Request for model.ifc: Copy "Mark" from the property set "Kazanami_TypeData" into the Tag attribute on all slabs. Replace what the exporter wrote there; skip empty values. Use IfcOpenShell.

First a look at what the model holds.

```python
import ifcopenshell
import ifcopenshell.util.element

model = ifcopenshell.open("model.ifc")
print(model.schema)
slabs = model.by_type("IfcSlab")
print(len(slabs), "slabs")
for e in slabs[:8]:
    source = ifcopenshell.util.element.get_pset(e, "Kazanami_TypeData", "Mark")
    target = e.Tag
    print(e.id(), repr(source), repr(target), sep=" | ")
```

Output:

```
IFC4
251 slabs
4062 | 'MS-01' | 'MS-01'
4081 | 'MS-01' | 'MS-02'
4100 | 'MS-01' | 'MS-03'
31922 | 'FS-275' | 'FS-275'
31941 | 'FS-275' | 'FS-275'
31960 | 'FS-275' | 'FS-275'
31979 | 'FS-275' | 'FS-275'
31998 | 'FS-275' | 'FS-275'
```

```python
import ifcopenshell
import ifcopenshell.util.element

model = ifcopenshell.open("model.ifc")

count = 0
for e in model.by_type("IfcSlab"):
    value = ifcopenshell.util.element.get_pset(e, "Kazanami_TypeData", "Mark")
    current = e.Tag
    if not value or not value.strip() or current == value:
        continue
    e.Tag = value
    count += 1

print(count, "slabs updated")

model.write("model_edited.ifc")
```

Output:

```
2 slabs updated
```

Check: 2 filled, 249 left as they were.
